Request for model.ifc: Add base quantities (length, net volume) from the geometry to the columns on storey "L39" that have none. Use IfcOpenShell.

First a look at what the model holds.

```python
import ifcopenshell
import ifcopenshell.util.element
import ifcopenshell.util.unit

model = ifcopenshell.open("model.ifc")
print(model.schema)
for unit_type in ("LENGTHUNIT", "AREAUNIT", "VOLUMEUNIT"):
    print(unit_type, ifcopenshell.util.unit.calculate_unit_scale(model, unit_type))
storey = next(s for s in model.by_type("IfcBuildingStorey") if s.Name == "L39")
columns = [e for e in ifcopenshell.util.element.get_decomposition(storey) if e.is_a("IfcColumn")]
for e in sorted(columns, key=lambda e: e.id()):
    print(e.id(), e.is_a(), e.Name, list(ifcopenshell.util.element.get_psets(e, qtos_only=True)), sep=" | ")
```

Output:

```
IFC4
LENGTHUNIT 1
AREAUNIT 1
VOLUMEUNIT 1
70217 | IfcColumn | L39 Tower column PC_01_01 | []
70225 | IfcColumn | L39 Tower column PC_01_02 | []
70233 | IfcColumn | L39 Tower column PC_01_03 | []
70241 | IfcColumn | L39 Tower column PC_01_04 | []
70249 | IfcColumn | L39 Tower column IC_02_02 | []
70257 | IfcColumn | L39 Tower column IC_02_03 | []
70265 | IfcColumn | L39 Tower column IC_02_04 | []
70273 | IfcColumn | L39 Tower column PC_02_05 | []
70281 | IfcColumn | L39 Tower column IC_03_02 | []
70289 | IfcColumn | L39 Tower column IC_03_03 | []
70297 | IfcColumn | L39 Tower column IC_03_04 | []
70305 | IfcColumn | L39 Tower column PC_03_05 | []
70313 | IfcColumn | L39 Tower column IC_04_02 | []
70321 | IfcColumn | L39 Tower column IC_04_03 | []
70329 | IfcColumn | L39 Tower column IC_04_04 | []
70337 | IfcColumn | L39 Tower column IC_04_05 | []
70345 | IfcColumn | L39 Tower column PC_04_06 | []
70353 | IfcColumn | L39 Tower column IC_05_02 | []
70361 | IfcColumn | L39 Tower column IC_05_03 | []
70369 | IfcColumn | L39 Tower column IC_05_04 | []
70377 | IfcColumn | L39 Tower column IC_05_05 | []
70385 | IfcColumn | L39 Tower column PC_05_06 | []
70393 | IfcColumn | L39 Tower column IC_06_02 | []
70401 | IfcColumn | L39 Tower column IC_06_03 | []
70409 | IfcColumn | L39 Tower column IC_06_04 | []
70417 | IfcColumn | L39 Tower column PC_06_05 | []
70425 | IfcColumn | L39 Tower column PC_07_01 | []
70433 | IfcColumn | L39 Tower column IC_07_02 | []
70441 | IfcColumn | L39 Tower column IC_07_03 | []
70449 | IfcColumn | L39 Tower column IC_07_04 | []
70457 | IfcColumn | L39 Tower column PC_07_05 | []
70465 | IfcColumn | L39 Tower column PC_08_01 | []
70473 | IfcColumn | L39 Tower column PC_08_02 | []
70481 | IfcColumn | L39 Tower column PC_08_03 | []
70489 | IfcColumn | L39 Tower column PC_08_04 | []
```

```python
import ifcopenshell
import ifcopenshell.api.pset
import ifcopenshell.geom
import ifcopenshell.util.element
import ifcopenshell.util.shape
import ifcopenshell.util.unit

model = ifcopenshell.open("model.ifc")
unit_scale = ifcopenshell.util.unit.calculate_unit_scale(model)
volume_scale = ifcopenshell.util.unit.calculate_unit_scale(model, "VOLUMEUNIT")
settings = ifcopenshell.geom.settings()

storey = next(s for s in model.by_type("IfcBuildingStorey") if s.Name == "L39")
columns = [e for e in ifcopenshell.util.element.get_decomposition(storey) if e.is_a("IfcColumn")]

for e in sorted(columns, key=lambda e: e.id()):
    if ifcopenshell.util.element.get_psets(e, qtos_only=True, should_inherit=False):
        continue
    # Geometry comes back in metres, in the element's own axes.
    shape = ifcopenshell.geom.create_shape(settings, e)
    values = {
        "Length": ifcopenshell.util.shape.get_z(shape.geometry) / unit_scale,
        "NetVolume": ifcopenshell.util.shape.get_volume(shape.geometry) / volume_scale,
    }
    qto = ifcopenshell.api.pset.add_qto(model, product=e, name="Qto_ColumnBaseQuantities")
    ifcopenshell.api.pset.edit_qto(model, qto=qto, properties=values)
    print(e.id(), {k: round(v, 3) for k, v in values.items()})

model.write("model_v2.ifc")
```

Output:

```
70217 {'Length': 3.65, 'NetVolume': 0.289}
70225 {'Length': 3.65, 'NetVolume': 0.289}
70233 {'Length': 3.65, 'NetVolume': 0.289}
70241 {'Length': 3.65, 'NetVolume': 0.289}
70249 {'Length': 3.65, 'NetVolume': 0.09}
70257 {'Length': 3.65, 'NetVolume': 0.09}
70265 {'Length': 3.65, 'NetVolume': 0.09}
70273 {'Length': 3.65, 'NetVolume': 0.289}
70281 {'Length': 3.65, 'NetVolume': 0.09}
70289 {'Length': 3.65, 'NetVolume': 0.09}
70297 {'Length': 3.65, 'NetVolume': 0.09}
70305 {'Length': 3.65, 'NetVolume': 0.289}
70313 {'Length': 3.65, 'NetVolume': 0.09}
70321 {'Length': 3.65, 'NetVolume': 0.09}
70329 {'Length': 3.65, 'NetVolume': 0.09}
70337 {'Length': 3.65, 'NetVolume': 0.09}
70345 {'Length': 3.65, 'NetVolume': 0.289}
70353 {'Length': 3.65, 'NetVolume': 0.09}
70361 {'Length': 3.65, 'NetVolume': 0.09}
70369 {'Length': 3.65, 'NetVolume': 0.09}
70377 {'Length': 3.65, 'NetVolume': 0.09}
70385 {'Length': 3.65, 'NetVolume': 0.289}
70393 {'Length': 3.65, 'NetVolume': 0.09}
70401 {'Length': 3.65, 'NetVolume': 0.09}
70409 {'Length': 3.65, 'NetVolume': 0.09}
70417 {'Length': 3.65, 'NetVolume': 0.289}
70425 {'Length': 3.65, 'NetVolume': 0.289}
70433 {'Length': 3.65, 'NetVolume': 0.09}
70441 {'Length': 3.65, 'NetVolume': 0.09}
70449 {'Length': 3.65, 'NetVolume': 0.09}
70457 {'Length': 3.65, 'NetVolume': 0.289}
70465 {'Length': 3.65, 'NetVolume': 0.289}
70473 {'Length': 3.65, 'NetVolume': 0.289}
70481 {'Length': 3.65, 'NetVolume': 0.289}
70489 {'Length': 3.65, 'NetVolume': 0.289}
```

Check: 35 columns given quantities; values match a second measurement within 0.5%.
